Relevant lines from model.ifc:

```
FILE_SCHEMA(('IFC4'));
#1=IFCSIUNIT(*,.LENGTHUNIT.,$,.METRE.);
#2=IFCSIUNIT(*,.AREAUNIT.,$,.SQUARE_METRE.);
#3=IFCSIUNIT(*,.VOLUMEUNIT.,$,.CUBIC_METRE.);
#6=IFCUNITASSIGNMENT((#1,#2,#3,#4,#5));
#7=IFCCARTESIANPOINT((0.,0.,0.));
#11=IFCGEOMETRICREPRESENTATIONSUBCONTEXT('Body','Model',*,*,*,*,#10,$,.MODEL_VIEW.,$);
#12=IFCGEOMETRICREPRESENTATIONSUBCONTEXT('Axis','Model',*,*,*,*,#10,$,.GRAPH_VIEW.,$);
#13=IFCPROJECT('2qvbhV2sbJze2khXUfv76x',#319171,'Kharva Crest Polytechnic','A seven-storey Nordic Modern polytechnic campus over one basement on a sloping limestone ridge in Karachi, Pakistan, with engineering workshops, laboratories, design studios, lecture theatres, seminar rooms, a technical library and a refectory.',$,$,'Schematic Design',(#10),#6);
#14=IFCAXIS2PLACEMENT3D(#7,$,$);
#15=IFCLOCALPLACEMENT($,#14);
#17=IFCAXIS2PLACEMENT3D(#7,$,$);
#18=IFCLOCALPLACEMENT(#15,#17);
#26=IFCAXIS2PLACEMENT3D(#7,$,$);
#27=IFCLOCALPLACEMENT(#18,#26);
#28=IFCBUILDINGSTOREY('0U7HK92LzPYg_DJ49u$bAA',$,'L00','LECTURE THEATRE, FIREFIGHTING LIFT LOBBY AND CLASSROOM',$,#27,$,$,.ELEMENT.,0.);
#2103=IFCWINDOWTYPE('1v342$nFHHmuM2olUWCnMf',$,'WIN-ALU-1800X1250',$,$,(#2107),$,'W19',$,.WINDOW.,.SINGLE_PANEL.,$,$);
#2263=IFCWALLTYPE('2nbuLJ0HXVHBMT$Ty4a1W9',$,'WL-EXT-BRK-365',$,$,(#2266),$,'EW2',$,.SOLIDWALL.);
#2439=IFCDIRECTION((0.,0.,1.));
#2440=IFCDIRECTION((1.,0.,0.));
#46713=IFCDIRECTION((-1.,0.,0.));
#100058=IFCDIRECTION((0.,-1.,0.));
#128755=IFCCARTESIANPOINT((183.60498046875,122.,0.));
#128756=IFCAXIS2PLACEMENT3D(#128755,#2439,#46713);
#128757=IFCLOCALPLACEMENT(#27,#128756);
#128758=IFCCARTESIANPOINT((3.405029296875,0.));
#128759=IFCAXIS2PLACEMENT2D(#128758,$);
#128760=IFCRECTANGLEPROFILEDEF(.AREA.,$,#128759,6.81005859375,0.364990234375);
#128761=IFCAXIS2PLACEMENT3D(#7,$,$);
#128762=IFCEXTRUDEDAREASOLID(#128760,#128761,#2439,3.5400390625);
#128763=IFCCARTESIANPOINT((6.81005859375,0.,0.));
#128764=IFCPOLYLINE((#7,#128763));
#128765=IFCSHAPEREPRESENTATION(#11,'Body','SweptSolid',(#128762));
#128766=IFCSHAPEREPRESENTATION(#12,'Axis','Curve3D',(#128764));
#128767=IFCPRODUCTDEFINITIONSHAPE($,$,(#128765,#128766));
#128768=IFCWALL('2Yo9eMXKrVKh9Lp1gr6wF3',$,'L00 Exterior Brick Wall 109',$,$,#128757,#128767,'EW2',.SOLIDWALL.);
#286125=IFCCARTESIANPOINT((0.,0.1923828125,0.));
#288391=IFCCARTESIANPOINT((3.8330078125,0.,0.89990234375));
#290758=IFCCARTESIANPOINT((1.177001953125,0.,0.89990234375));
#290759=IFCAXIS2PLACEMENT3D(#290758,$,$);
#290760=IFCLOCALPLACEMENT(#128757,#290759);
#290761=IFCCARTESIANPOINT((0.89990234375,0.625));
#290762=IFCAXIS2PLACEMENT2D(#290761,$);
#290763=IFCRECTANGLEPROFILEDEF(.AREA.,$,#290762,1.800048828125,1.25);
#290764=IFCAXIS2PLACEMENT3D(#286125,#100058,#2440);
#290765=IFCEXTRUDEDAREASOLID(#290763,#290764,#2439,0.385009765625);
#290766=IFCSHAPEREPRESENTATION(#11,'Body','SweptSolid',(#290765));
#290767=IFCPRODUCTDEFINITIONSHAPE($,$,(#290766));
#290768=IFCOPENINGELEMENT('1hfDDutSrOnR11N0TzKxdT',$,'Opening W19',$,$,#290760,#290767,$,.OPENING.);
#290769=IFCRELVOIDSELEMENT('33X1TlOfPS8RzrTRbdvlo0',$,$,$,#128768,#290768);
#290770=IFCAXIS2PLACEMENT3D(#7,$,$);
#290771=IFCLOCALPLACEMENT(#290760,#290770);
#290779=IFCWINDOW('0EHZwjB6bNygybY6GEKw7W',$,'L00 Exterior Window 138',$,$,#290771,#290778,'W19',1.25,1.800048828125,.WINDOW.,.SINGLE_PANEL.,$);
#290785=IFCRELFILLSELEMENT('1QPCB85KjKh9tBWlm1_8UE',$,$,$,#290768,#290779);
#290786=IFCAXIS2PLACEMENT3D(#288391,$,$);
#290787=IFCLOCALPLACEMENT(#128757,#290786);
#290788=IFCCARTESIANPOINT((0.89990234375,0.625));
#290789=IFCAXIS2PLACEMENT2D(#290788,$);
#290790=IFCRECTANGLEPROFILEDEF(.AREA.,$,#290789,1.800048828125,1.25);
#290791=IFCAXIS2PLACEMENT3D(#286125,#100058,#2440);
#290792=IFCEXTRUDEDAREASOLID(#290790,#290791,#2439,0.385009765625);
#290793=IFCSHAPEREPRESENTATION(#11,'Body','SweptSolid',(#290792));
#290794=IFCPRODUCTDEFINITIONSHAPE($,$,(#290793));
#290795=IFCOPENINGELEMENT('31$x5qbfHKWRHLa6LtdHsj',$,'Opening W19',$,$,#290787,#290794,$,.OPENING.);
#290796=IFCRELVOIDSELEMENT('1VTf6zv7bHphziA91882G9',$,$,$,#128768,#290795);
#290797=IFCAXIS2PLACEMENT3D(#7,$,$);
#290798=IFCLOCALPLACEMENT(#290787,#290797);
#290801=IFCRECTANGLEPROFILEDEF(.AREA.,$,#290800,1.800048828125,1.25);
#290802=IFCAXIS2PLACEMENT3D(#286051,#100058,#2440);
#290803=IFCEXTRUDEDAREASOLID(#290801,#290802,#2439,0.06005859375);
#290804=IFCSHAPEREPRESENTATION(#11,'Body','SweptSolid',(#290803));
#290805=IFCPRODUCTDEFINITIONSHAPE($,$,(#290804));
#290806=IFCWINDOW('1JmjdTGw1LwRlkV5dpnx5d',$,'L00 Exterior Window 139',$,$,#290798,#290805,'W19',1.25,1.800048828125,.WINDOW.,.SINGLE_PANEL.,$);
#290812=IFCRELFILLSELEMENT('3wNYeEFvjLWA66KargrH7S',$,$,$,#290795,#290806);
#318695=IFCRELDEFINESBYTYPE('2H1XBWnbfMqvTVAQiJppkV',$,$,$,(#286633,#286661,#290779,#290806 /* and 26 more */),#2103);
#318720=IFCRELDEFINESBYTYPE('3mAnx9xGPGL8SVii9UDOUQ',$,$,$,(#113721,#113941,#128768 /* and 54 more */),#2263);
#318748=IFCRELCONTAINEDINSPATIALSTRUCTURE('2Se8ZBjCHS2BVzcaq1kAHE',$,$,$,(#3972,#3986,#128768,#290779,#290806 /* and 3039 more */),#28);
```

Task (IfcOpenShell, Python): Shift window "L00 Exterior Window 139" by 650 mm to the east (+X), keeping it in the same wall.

```python
import ifcopenshell
import ifcopenshell.api.geometry
import ifcopenshell.util.placement
import ifcopenshell.util.unit

model = ifcopenshell.open("model.ifc")
unit_scale = ifcopenshell.util.unit.calculate_unit_scale(model)

window = model.by_guid("1JmjdTGw1LwRlkV5dpnx5d")
opening = window.FillsVoids[0].RelatingOpeningElement
wall = opening.VoidsElements[0].RelatingBuildingElement

wall_matrix = ifcopenshell.util.placement.get_local_placement(wall.ObjectPlacement)
shift = wall_matrix[:3, 0] * -0.65 / unit_scale
before = ifcopenshell.util.placement.get_local_placement(window.ObjectPlacement)[:3, 3].copy()

# The window is placed relative to its opening, so it follows when the opening moves.
matrix = ifcopenshell.util.placement.get_local_placement(opening.ObjectPlacement)
matrix[:3, 3] += shift
ifcopenshell.api.geometry.edit_object_placement(
    model, product=opening, matrix=matrix, is_si=False, should_transform_children=True
)

after = ifcopenshell.util.placement.get_local_placement(window.ObjectPlacement)[:3, 3]
print("window moved by", (after - before).round(3) + 0.0)

model.write("model_rev.ifc")
```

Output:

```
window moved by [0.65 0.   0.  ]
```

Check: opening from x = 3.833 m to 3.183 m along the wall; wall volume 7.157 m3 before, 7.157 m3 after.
